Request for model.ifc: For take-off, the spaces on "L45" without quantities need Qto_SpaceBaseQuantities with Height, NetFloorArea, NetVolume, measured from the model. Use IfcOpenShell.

First a look at what the model holds.

```python
import ifcopenshell
import ifcopenshell.util.element
import ifcopenshell.util.unit

model = ifcopenshell.open("model.ifc")
print(model.schema)
for unit_type in ("LENGTHUNIT", "AREAUNIT", "VOLUMEUNIT"):
    print(unit_type, ifcopenshell.util.unit.calculate_unit_scale(model, unit_type))
storey = next(s for s in model.by_type("IfcBuildingStorey") if s.Name == "L45")
spaces = [e for e in ifcopenshell.util.element.get_decomposition(storey) if e.is_a("IfcSpace")]
for e in sorted(spaces, key=lambda e: e.id()):
    print(e.id(), e.is_a(), e.Name, list(ifcopenshell.util.element.get_psets(e, qtos_only=True)), sep=" | ")
```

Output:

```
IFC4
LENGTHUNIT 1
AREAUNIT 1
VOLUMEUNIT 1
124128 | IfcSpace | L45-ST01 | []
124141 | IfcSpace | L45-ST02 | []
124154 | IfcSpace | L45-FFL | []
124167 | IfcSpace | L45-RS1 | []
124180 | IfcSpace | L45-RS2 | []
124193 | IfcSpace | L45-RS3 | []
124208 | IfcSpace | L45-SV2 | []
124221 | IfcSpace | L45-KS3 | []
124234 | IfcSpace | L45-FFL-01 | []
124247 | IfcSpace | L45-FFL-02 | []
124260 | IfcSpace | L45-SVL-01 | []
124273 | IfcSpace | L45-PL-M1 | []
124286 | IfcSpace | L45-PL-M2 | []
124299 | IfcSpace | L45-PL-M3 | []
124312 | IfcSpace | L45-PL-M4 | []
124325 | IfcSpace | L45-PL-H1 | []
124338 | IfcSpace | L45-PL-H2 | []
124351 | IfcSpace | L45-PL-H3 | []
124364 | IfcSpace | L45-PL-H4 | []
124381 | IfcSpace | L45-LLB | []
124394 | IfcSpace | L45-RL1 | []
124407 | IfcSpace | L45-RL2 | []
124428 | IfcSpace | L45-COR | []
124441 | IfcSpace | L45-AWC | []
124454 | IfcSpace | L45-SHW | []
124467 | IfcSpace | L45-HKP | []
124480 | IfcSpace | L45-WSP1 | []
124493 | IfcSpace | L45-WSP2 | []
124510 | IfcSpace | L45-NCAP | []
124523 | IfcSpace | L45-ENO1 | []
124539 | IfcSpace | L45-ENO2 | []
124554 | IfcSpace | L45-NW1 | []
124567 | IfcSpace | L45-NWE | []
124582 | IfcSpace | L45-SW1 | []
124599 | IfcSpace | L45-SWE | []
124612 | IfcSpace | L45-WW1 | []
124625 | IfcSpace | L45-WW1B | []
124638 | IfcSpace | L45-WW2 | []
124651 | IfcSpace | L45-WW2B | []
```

```python
import ifcopenshell
import ifcopenshell.api.pset
import ifcopenshell.geom
import ifcopenshell.util.element
import ifcopenshell.util.shape
import ifcopenshell.util.unit

model = ifcopenshell.open("model.ifc")
unit_scale = ifcopenshell.util.unit.calculate_unit_scale(model)
area_scale = ifcopenshell.util.unit.calculate_unit_scale(model, "AREAUNIT")
volume_scale = ifcopenshell.util.unit.calculate_unit_scale(model, "VOLUMEUNIT")
settings = ifcopenshell.geom.settings()

storey = next(s for s in model.by_type("IfcBuildingStorey") if s.Name == "L45")
spaces = [e for e in ifcopenshell.util.element.get_decomposition(storey) if e.is_a("IfcSpace")]

for e in sorted(spaces, key=lambda e: e.id()):
    if ifcopenshell.util.element.get_psets(e, qtos_only=True, should_inherit=False):
        continue
    # Geometry comes back in metres, in the element's own axes.
    shape = ifcopenshell.geom.create_shape(settings, e)
    values = {
        "Height": ifcopenshell.util.shape.get_z(shape.geometry) / unit_scale,
        "NetFloorArea": ifcopenshell.util.shape.get_footprint_area(shape.geometry) / area_scale,
        "NetVolume": ifcopenshell.util.shape.get_volume(shape.geometry) / volume_scale,
    }
    qto = ifcopenshell.api.pset.add_qto(model, product=e, name="Qto_SpaceBaseQuantities")
    ifcopenshell.api.pset.edit_qto(model, qto=qto, properties=values)
    print(e.id(), {k: round(v, 3) for k, v in values.items()})

model.write("model_v2.ifc")
```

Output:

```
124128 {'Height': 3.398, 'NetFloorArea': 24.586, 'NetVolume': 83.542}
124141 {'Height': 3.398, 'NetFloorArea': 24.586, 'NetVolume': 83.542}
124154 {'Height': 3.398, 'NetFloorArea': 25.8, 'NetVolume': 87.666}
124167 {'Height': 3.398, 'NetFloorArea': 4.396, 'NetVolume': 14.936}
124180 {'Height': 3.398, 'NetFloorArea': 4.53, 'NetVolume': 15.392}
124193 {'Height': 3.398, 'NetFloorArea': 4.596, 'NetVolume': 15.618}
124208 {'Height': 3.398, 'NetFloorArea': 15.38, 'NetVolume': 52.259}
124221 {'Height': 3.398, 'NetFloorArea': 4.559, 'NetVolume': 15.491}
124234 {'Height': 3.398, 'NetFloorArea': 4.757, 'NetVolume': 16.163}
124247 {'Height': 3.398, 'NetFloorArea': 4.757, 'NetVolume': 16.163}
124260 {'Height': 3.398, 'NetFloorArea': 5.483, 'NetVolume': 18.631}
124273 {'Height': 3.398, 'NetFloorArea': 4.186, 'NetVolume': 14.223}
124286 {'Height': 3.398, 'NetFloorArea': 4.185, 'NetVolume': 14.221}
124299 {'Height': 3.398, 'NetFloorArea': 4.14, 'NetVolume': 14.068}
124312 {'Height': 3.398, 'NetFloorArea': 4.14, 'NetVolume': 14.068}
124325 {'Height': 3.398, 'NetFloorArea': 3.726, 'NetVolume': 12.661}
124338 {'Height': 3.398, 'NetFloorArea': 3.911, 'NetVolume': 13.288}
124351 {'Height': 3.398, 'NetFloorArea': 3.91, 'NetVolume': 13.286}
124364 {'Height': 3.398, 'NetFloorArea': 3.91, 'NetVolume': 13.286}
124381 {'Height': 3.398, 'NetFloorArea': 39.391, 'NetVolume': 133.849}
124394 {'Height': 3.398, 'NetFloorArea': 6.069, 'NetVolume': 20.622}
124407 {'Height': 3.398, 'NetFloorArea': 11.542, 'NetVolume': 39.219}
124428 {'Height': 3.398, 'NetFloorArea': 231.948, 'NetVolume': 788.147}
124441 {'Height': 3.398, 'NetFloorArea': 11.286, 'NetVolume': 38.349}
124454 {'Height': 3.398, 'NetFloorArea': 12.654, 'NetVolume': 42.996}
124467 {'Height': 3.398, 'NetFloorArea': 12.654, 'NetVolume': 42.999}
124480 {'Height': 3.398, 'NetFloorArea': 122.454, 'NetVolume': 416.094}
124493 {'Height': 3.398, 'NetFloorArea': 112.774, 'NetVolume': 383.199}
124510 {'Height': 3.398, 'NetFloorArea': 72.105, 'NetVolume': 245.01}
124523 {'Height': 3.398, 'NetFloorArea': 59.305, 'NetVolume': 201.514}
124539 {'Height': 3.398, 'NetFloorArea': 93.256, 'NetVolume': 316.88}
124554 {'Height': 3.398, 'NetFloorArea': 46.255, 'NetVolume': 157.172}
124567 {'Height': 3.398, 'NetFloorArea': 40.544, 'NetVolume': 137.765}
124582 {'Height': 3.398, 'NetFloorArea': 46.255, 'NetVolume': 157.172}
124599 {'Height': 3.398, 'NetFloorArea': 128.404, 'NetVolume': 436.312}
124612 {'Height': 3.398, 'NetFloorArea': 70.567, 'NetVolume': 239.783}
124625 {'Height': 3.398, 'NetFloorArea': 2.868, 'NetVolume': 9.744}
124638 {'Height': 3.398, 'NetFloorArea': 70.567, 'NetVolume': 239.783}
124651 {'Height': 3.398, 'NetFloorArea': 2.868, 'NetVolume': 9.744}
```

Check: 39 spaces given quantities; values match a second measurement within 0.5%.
